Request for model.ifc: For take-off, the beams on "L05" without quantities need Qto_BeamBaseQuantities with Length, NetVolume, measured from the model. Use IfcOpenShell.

First a look at what the model holds.

```python
import ifcopenshell
import ifcopenshell.util.element
import ifcopenshell.util.unit

model = ifcopenshell.open("model.ifc")
print(model.schema)
for unit_type in ("LENGTHUNIT", "AREAUNIT", "VOLUMEUNIT"):
    print(unit_type, ifcopenshell.util.unit.calculate_unit_scale(model, unit_type))
storey = next(s for s in model.by_type("IfcBuildingStorey") if s.Name == "L05")
beams = [e for e in ifcopenshell.util.element.get_decomposition(storey) if e.is_a("IfcBeam")]
for e in sorted(beams, key=lambda e: e.id()):
    print(e.id(), e.is_a(), e.Name, list(ifcopenshell.util.element.get_psets(e, qtos_only=True)), sep=" | ")
```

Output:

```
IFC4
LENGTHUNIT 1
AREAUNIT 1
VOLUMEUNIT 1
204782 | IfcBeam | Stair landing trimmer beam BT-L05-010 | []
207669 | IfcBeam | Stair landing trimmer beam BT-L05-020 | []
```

```python
import ifcopenshell
import ifcopenshell.api.pset
import ifcopenshell.geom
import ifcopenshell.util.element
import ifcopenshell.util.shape
import ifcopenshell.util.unit

model = ifcopenshell.open("model.ifc")
unit_scale = ifcopenshell.util.unit.calculate_unit_scale(model)
volume_scale = ifcopenshell.util.unit.calculate_unit_scale(model, "VOLUMEUNIT")
settings = ifcopenshell.geom.settings()

storey = next(s for s in model.by_type("IfcBuildingStorey") if s.Name == "L05")
beams = [e for e in ifcopenshell.util.element.get_decomposition(storey) if e.is_a("IfcBeam")]

for e in sorted(beams, key=lambda e: e.id()):
    if ifcopenshell.util.element.get_psets(e, qtos_only=True, should_inherit=False):
        continue
    # Geometry comes back in metres, in the element's own axes.
    shape = ifcopenshell.geom.create_shape(settings, e)
    values = {
        "Length": ifcopenshell.util.shape.get_max_xyz(shape.geometry) / unit_scale,
        "NetVolume": ifcopenshell.util.shape.get_volume(shape.geometry) / volume_scale,
    }
    qto = ifcopenshell.api.pset.add_qto(model, product=e, name="Qto_BeamBaseQuantities")
    ifcopenshell.api.pset.edit_qto(model, qto=qto, properties=values)
    print(e.id(), {k: round(v, 3) for k, v in values.items()})

model.write("model_rev.ifc")
```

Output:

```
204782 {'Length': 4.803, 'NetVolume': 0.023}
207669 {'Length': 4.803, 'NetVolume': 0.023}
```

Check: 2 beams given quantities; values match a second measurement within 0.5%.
